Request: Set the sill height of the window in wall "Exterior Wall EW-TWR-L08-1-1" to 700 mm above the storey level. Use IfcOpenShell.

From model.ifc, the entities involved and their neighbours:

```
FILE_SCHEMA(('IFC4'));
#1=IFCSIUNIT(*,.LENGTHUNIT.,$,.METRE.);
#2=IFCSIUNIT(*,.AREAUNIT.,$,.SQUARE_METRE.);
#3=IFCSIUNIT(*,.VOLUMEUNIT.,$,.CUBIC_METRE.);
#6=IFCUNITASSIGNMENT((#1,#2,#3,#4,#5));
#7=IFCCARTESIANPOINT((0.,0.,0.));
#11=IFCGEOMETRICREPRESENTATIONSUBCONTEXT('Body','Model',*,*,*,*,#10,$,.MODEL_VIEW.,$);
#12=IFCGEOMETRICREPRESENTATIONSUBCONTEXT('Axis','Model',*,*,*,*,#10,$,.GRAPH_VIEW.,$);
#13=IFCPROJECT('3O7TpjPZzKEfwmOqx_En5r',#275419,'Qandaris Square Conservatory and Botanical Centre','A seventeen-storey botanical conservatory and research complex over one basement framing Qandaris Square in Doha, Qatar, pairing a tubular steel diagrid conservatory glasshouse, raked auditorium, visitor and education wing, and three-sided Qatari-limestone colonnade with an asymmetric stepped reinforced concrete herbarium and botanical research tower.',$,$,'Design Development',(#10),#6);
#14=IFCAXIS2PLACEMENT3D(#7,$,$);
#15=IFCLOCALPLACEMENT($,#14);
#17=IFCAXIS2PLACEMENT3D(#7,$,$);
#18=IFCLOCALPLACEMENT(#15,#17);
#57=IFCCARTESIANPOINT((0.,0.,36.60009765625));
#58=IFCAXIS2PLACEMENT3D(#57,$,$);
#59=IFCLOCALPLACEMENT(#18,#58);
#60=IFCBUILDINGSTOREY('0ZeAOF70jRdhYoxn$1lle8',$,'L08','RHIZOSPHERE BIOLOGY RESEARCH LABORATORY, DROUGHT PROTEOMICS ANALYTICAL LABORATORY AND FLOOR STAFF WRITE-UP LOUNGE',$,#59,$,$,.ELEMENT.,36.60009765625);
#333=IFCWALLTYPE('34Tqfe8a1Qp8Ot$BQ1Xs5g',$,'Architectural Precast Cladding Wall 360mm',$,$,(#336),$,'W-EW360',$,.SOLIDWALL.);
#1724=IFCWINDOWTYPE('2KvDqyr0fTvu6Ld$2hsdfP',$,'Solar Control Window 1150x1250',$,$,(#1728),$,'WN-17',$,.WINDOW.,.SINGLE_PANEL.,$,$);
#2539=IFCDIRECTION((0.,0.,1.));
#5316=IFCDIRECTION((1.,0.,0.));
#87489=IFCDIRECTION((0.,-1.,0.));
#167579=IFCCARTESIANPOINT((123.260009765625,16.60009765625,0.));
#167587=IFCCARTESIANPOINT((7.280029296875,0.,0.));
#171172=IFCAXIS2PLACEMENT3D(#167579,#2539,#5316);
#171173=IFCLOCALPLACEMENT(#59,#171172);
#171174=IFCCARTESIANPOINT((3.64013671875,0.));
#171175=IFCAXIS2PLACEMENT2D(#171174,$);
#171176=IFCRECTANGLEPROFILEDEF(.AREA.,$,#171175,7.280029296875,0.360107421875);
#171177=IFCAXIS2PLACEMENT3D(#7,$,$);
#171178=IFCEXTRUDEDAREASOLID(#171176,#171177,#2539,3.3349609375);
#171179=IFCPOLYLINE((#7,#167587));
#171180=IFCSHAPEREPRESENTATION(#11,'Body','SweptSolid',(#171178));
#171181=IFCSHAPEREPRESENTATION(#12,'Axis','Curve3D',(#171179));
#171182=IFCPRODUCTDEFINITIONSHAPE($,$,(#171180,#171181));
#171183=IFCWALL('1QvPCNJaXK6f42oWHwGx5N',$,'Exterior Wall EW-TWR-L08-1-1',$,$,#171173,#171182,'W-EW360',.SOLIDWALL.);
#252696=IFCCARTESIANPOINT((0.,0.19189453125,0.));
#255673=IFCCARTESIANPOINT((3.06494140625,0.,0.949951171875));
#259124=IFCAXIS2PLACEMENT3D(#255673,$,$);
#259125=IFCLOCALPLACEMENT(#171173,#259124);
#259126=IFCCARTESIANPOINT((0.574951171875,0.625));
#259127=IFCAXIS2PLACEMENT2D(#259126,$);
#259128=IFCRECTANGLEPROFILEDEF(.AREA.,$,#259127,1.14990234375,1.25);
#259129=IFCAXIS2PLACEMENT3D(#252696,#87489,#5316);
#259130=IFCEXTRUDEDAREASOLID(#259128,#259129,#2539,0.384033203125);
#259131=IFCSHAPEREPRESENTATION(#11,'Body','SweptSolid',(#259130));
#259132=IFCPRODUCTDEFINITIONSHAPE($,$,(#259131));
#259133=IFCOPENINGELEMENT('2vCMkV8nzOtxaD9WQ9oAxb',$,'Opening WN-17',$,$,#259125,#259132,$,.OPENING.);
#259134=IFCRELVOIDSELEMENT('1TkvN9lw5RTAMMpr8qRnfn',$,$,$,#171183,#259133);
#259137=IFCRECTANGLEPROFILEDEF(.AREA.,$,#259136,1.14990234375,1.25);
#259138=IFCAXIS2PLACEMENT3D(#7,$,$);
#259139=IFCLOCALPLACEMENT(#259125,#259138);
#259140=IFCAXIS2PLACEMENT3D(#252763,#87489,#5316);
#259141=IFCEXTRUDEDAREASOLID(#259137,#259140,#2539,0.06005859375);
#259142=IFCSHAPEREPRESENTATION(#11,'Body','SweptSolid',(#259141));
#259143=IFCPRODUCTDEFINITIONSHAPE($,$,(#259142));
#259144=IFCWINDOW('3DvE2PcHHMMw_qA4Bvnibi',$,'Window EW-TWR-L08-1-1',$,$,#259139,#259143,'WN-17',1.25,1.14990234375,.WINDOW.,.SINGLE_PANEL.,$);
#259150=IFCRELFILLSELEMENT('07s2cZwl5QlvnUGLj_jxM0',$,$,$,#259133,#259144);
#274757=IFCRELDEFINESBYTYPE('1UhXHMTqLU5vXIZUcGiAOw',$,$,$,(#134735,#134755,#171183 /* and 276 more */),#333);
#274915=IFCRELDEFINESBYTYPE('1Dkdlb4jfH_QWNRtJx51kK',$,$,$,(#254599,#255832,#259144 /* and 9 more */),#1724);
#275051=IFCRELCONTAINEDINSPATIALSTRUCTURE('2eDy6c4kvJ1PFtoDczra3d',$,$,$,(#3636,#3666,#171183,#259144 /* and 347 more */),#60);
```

```python
import numpy as np
import ifcopenshell
import ifcopenshell.api.geometry
import ifcopenshell.geom
import ifcopenshell.util.element
import ifcopenshell.util.placement
import ifcopenshell.util.shape
import ifcopenshell.util.unit

model = ifcopenshell.open("model.ifc")
unit_scale = ifcopenshell.util.unit.calculate_unit_scale(model)

window = model.by_guid("3DvE2PcHHMMw_qA4Bvnibi")
opening = window.FillsVoids[0].RelatingOpeningElement
storey = ifcopenshell.util.element.get_container(window, ifc_class="IfcBuildingStorey")
level = ifcopenshell.util.placement.get_local_placement(storey.ObjectPlacement)[2, 3]

# The opening's origin need not be at the sill, so measure its lowest point.
shape = ifcopenshell.geom.create_shape(ifcopenshell.geom.settings(), opening)
bottom = ifcopenshell.util.shape.get_shape_bottom_elevation(shape, shape.geometry) / unit_scale
dz = level + 0.7 - bottom

shift = np.array([0.0, 0.0, dz])
# The window is placed relative to its opening, so it follows when the opening moves.
matrix = ifcopenshell.util.placement.get_local_placement(opening.ObjectPlacement)
matrix[:3, 3] += shift
ifcopenshell.api.geometry.edit_object_placement(
    model, product=opening, matrix=matrix, is_si=False, should_transform_children=True
)

print(f"moved by {dz * unit_scale:+.3f} m")

model.write("model_rev.ifc")
```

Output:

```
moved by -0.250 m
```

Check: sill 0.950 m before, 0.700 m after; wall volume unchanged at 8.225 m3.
